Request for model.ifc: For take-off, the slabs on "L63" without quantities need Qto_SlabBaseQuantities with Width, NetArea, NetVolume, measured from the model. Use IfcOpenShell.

First a look at what the model holds.

```python
import ifcopenshell
import ifcopenshell.util.element
import ifcopenshell.util.unit

model = ifcopenshell.open("model.ifc")
print(model.schema)
for unit_type in ("LENGTHUNIT", "AREAUNIT", "VOLUMEUNIT"):
    print(unit_type, ifcopenshell.util.unit.calculate_unit_scale(model, unit_type))
storey = next(s for s in model.by_type("IfcBuildingStorey") if s.Name == "L63")
slabs = [e for e in ifcopenshell.util.element.get_decomposition(storey) if e.is_a("IfcSlab")]
for e in sorted(slabs, key=lambda e: e.id()):
    print(e.id(), e.is_a(), e.Name, list(ifcopenshell.util.element.get_psets(e, qtos_only=True)), sep=" | ")
```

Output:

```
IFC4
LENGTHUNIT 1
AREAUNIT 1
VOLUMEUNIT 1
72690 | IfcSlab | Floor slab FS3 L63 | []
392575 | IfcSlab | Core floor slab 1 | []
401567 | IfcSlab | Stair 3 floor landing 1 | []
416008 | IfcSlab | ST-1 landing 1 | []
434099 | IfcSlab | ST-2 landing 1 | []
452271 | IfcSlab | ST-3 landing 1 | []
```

```python
import ifcopenshell
import ifcopenshell.api.pset
import ifcopenshell.geom
import ifcopenshell.util.element
import ifcopenshell.util.shape
import ifcopenshell.util.unit

model = ifcopenshell.open("model.ifc")
unit_scale = ifcopenshell.util.unit.calculate_unit_scale(model)
area_scale = ifcopenshell.util.unit.calculate_unit_scale(model, "AREAUNIT")
volume_scale = ifcopenshell.util.unit.calculate_unit_scale(model, "VOLUMEUNIT")
settings = ifcopenshell.geom.settings()

storey = next(s for s in model.by_type("IfcBuildingStorey") if s.Name == "L63")
slabs = [e for e in ifcopenshell.util.element.get_decomposition(storey) if e.is_a("IfcSlab")]

for e in sorted(slabs, key=lambda e: e.id()):
    if ifcopenshell.util.element.get_psets(e, qtos_only=True, should_inherit=False):
        continue
    # Geometry comes back in metres, in the element's own axes.
    shape = ifcopenshell.geom.create_shape(settings, e)
    values = {
        "Width": ifcopenshell.util.shape.get_z(shape.geometry) / unit_scale,
        "NetArea": ifcopenshell.util.shape.get_footprint_area(shape.geometry) / area_scale,
        "NetVolume": ifcopenshell.util.shape.get_volume(shape.geometry) / volume_scale,
    }
    qto = ifcopenshell.api.pset.add_qto(model, product=e, name="Qto_SlabBaseQuantities")
    ifcopenshell.api.pset.edit_qto(model, qto=qto, properties=values)
    print(e.id(), {k: round(v, 3) for k, v in values.items()})

model.write("model_edited.ifc")
```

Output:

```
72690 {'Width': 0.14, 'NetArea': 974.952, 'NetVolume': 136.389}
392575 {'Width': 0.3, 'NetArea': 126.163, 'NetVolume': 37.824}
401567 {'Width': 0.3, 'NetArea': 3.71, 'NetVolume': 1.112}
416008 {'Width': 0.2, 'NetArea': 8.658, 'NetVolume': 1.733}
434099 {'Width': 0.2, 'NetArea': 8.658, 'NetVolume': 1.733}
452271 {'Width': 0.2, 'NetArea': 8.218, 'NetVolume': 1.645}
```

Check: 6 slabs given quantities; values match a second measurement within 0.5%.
